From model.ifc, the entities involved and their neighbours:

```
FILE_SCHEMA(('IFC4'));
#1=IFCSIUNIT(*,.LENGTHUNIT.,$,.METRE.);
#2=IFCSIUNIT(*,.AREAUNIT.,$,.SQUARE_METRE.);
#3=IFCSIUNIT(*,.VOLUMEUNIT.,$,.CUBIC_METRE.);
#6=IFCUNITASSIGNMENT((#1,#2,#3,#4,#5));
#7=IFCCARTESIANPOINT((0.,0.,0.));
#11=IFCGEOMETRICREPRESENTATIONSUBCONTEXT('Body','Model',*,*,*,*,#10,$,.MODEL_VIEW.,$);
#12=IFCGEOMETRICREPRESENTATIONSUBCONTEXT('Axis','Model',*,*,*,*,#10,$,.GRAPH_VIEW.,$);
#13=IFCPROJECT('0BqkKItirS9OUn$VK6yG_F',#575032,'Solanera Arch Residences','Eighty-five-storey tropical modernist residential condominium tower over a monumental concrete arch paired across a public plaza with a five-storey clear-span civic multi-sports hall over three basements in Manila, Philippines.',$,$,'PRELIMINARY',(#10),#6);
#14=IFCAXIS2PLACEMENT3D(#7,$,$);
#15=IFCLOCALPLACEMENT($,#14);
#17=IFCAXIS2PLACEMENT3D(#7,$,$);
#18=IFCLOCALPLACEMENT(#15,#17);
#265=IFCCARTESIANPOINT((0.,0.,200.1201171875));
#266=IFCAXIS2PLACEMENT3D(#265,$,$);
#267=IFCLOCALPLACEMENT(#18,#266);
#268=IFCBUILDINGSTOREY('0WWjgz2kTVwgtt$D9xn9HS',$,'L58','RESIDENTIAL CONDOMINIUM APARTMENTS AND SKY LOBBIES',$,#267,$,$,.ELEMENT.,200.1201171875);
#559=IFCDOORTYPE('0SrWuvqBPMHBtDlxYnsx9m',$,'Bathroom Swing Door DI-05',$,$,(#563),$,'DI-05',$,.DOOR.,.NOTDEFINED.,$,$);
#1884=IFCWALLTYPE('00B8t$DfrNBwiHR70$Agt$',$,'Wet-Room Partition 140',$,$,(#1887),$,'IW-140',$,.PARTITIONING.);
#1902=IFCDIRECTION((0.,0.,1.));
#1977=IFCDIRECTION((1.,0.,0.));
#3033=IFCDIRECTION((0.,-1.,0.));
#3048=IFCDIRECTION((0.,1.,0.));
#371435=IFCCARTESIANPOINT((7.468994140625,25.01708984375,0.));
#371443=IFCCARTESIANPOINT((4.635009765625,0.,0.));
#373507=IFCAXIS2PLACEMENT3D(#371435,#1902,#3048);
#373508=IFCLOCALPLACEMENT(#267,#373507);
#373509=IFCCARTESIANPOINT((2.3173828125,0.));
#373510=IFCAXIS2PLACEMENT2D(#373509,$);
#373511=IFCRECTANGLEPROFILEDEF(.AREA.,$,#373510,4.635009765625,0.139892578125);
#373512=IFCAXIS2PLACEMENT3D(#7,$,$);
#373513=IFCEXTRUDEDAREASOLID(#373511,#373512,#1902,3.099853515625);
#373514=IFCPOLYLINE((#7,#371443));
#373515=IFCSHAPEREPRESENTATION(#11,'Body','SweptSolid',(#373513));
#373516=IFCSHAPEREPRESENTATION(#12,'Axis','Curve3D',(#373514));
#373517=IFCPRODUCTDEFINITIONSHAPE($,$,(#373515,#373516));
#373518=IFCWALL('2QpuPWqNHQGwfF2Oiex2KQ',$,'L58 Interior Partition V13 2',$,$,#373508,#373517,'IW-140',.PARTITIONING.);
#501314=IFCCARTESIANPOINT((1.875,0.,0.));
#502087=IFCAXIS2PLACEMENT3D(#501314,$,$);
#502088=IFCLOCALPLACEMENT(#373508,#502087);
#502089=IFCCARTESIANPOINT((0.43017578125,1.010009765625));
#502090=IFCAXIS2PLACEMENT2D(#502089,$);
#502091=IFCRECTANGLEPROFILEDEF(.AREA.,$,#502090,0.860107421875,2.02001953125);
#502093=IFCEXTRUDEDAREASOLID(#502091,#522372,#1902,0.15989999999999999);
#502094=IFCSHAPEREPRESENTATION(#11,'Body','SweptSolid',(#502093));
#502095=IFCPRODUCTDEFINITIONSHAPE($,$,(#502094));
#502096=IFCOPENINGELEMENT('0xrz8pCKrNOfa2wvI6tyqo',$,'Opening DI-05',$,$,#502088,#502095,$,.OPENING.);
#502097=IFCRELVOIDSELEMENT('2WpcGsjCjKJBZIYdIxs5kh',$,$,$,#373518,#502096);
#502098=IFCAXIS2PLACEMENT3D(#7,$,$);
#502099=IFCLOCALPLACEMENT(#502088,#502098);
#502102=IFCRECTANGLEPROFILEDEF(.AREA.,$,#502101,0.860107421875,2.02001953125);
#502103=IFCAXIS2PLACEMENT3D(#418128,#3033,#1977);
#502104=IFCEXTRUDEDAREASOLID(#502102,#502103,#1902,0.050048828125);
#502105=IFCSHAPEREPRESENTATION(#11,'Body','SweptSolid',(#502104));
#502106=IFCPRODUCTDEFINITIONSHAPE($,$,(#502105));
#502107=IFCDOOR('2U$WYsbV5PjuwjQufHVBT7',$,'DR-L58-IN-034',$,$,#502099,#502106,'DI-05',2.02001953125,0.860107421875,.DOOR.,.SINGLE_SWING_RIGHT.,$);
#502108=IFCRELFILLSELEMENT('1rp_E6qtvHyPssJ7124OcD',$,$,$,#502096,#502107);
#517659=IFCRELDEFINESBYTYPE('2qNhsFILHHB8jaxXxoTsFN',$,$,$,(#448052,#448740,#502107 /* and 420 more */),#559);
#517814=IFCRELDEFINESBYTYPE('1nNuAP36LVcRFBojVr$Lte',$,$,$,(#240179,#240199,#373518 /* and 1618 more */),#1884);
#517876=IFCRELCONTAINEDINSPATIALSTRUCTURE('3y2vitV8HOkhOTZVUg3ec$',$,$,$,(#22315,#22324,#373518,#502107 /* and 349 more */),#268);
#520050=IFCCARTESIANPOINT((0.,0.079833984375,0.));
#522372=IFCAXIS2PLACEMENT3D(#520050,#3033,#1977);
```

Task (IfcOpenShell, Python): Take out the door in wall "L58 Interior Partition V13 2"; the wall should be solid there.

```python
import ifcopenshell
import ifcopenshell.api.feature
import ifcopenshell.api.root
import ifcopenshell.geom
import ifcopenshell.util.shape

model = ifcopenshell.open("model.ifc")
settings = ifcopenshell.geom.settings()


def volume(element):
    """Net volume in cubic metres, openings subtracted."""
    shape = ifcopenshell.geom.create_shape(settings, element)
    return ifcopenshell.util.shape.get_volume(shape.geometry)


door = model.by_guid("2U$WYsbV5PjuwjQufHVBT7")
opening = door.FillsVoids[0].RelatingOpeningElement
wall = opening.VoidsElements[0].RelatingBuildingElement
before = volume(wall)

ifcopenshell.api.root.remove_product(model, product=door)
ifcopenshell.api.feature.remove_feature(model, feature=opening)

after = volume(wall)

print(f"wall volume {before:.3f} -> {after:.3f} m3")

model.write("model_v2.ifc")
```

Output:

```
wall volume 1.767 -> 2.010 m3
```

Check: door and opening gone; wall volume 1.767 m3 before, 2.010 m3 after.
